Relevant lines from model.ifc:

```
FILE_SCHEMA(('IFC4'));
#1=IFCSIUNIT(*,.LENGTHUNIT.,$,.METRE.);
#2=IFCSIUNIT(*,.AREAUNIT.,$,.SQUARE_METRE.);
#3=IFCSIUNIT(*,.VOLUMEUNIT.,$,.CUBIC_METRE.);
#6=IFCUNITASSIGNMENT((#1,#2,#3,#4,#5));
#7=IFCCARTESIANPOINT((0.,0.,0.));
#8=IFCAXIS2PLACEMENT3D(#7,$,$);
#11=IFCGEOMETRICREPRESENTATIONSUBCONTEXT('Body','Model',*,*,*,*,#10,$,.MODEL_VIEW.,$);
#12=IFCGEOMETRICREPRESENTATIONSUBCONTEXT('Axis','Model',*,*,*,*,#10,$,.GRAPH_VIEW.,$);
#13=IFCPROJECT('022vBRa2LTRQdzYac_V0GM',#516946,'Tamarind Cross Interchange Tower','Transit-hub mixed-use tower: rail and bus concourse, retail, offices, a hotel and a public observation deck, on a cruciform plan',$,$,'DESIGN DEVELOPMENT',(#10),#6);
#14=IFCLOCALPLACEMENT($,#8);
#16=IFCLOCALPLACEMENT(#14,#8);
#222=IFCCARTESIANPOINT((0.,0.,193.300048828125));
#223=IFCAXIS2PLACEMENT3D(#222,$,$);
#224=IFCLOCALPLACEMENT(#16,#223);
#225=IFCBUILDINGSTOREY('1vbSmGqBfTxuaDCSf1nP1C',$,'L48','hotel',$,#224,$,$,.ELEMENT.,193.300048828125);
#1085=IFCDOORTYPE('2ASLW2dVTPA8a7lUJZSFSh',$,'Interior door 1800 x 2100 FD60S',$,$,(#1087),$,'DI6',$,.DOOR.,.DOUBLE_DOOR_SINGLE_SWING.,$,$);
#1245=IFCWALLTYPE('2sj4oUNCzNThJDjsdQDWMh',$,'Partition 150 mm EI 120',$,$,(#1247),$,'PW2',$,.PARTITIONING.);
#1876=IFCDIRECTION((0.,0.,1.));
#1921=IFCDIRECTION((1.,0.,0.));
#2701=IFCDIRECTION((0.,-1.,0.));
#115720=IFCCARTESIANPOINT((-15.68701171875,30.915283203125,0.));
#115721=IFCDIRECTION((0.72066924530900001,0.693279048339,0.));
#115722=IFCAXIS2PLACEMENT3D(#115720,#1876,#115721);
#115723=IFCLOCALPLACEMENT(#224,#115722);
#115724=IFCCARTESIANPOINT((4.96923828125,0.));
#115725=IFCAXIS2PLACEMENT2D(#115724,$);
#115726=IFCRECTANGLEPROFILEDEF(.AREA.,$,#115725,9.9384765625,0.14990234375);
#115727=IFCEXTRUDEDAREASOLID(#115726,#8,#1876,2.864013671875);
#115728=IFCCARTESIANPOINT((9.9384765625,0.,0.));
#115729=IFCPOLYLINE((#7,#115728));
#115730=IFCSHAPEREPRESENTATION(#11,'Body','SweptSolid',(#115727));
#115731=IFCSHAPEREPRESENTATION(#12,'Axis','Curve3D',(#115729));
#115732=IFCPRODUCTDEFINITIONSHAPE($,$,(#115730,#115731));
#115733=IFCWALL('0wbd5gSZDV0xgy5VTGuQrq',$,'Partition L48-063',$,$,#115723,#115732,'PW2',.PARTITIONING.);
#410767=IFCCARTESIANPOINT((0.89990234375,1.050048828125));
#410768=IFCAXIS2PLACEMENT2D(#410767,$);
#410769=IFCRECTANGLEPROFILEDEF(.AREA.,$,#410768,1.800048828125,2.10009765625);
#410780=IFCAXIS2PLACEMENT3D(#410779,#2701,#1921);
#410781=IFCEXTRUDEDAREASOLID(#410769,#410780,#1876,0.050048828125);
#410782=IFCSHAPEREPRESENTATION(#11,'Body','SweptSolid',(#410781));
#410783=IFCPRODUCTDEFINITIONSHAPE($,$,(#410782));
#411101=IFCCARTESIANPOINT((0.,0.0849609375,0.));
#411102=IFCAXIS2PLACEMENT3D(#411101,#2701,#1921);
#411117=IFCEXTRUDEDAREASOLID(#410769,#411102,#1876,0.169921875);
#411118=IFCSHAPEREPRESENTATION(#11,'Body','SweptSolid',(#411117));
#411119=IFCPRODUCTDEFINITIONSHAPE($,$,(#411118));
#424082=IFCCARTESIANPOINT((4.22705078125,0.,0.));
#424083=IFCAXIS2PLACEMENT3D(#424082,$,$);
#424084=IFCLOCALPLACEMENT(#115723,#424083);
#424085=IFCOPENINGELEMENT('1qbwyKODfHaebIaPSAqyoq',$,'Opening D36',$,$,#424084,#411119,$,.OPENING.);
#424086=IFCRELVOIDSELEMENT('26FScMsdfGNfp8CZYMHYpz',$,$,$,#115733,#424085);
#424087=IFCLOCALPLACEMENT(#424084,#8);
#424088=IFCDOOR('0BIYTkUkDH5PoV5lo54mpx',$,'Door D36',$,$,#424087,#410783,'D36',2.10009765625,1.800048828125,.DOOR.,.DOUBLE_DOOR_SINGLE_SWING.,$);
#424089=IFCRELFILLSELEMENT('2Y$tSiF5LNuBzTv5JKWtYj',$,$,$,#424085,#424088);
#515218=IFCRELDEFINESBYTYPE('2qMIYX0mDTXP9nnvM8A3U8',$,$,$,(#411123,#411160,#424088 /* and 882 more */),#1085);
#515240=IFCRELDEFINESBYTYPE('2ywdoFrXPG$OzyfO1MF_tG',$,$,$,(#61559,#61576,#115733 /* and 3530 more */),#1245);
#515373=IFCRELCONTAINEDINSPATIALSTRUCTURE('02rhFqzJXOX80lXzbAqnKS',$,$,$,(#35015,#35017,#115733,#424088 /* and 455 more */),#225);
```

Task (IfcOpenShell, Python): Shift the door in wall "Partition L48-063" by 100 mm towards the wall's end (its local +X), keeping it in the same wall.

```python
import ifcopenshell
import ifcopenshell.api.geometry
import ifcopenshell.util.placement
import ifcopenshell.util.unit

model = ifcopenshell.open("model.ifc")
unit_scale = ifcopenshell.util.unit.calculate_unit_scale(model)

door = model.by_guid("0BIYTkUkDH5PoV5lo54mpx")
opening = door.FillsVoids[0].RelatingOpeningElement
wall = opening.VoidsElements[0].RelatingBuildingElement

wall_matrix = ifcopenshell.util.placement.get_local_placement(wall.ObjectPlacement)
shift = wall_matrix[:3, 0] * 0.1 / unit_scale
before = ifcopenshell.util.placement.get_local_placement(door.ObjectPlacement)[:3, 3].copy()

# The door is placed relative to its opening, so it follows when the opening moves.
matrix = ifcopenshell.util.placement.get_local_placement(opening.ObjectPlacement)
matrix[:3, 3] += shift
ifcopenshell.api.geometry.edit_object_placement(
    model, product=opening, matrix=matrix, is_si=False, should_transform_children=True
)

after = ifcopenshell.util.placement.get_local_placement(door.ObjectPlacement)[:3, 3]
print("door moved by", (after - before).round(3) + 0.0)

model.write("model_v2.ifc")
```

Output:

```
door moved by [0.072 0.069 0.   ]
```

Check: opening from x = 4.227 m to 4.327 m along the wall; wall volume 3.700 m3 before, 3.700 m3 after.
